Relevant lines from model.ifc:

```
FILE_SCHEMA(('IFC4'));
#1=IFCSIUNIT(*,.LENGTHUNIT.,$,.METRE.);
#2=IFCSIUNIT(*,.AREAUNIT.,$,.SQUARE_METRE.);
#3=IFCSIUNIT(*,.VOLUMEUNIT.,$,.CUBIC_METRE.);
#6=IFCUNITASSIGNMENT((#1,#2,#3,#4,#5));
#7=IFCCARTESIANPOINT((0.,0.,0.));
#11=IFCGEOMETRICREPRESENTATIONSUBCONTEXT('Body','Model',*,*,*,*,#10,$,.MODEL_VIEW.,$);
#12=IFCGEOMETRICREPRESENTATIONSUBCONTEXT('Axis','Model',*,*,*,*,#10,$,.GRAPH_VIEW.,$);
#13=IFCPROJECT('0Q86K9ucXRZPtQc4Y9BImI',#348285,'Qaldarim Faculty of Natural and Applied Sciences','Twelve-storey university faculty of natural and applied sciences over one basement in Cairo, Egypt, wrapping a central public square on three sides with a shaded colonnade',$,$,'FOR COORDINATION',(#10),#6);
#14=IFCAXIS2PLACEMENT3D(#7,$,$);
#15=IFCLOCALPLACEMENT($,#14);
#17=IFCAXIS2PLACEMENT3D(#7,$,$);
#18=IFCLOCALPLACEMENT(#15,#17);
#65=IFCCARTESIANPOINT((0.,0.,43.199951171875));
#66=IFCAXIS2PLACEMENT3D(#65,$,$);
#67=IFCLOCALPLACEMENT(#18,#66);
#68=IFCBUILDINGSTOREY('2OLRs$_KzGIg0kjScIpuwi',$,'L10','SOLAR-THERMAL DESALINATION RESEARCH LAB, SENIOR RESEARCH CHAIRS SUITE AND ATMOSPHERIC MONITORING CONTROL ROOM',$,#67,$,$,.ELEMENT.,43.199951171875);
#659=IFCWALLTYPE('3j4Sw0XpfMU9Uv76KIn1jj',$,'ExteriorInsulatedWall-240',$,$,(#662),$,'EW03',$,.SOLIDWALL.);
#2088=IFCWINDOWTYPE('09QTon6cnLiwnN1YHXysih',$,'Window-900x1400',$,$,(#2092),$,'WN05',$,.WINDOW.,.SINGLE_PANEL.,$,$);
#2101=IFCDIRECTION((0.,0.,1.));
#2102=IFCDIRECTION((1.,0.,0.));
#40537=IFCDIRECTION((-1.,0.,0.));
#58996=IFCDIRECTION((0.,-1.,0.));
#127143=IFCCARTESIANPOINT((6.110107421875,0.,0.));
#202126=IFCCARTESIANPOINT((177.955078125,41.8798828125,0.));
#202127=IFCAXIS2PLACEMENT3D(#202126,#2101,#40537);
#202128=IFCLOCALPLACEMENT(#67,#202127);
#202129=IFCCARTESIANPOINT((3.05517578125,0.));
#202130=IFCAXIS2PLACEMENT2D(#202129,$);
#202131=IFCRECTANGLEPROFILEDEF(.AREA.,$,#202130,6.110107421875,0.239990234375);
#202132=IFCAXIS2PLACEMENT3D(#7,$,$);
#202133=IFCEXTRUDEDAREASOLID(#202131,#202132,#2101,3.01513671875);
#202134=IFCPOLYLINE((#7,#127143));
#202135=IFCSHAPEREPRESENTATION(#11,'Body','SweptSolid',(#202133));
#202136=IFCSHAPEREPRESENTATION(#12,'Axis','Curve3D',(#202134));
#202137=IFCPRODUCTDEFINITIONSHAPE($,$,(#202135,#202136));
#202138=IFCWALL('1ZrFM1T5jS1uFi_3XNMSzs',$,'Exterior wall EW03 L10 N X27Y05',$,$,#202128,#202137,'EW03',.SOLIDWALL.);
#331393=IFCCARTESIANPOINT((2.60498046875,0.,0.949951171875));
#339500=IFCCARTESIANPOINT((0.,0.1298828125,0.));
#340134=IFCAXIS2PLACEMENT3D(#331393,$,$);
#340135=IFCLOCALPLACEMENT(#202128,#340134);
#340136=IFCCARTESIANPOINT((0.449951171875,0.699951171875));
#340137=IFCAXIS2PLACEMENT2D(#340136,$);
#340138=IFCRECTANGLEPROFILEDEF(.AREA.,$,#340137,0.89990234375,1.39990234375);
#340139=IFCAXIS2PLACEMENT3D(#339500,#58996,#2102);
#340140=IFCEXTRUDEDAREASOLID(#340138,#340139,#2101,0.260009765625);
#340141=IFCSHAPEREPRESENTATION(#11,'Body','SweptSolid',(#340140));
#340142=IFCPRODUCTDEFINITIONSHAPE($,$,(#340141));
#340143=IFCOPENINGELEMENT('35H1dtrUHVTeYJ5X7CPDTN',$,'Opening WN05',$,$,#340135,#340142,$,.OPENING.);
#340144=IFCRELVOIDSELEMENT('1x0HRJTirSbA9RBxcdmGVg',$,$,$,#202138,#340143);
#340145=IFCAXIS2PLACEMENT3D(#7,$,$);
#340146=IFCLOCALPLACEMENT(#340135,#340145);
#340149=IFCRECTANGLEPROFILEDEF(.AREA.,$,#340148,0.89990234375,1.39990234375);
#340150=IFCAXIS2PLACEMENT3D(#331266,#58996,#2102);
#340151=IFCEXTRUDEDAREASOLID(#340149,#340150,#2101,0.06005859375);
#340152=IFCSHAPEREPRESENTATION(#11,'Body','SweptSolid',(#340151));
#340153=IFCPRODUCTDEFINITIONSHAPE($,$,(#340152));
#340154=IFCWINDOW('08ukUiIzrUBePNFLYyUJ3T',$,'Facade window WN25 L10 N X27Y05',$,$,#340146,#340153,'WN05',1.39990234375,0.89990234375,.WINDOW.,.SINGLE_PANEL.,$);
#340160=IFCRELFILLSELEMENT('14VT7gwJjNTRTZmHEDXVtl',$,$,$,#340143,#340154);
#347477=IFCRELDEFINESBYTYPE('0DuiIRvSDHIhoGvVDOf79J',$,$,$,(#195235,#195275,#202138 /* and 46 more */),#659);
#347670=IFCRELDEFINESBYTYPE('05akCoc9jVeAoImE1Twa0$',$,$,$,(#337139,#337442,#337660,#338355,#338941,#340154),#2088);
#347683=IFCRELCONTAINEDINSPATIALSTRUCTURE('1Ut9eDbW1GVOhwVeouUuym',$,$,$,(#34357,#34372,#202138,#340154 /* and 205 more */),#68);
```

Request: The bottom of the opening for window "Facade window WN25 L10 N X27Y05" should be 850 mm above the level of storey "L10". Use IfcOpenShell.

```python
import numpy as np
import ifcopenshell
import ifcopenshell.api.geometry
import ifcopenshell.geom
import ifcopenshell.util.element
import ifcopenshell.util.placement
import ifcopenshell.util.shape
import ifcopenshell.util.unit

model = ifcopenshell.open("model.ifc")
unit_scale = ifcopenshell.util.unit.calculate_unit_scale(model)

window = model.by_guid("08ukUiIzrUBePNFLYyUJ3T")
opening = window.FillsVoids[0].RelatingOpeningElement
storey = ifcopenshell.util.element.get_container(window, ifc_class="IfcBuildingStorey")
level = ifcopenshell.util.placement.get_local_placement(storey.ObjectPlacement)[2, 3]

# The opening's origin need not be at the sill, so measure its lowest point.
shape = ifcopenshell.geom.create_shape(ifcopenshell.geom.settings(), opening)
bottom = ifcopenshell.util.shape.get_shape_bottom_elevation(shape, shape.geometry) / unit_scale
dz = level + 0.85 / unit_scale - bottom

shift = np.array([0.0, 0.0, dz])
# The window is placed relative to its opening, so it follows when the opening moves.
matrix = ifcopenshell.util.placement.get_local_placement(opening.ObjectPlacement)
matrix[:3, 3] += shift
ifcopenshell.api.geometry.edit_object_placement(
    model, product=opening, matrix=matrix, is_si=False, should_transform_children=True
)

print(f"moved by {dz * unit_scale:+.3f} m")

model.write("model_edited.ifc")
```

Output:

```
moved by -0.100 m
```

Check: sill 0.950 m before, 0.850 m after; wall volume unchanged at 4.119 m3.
